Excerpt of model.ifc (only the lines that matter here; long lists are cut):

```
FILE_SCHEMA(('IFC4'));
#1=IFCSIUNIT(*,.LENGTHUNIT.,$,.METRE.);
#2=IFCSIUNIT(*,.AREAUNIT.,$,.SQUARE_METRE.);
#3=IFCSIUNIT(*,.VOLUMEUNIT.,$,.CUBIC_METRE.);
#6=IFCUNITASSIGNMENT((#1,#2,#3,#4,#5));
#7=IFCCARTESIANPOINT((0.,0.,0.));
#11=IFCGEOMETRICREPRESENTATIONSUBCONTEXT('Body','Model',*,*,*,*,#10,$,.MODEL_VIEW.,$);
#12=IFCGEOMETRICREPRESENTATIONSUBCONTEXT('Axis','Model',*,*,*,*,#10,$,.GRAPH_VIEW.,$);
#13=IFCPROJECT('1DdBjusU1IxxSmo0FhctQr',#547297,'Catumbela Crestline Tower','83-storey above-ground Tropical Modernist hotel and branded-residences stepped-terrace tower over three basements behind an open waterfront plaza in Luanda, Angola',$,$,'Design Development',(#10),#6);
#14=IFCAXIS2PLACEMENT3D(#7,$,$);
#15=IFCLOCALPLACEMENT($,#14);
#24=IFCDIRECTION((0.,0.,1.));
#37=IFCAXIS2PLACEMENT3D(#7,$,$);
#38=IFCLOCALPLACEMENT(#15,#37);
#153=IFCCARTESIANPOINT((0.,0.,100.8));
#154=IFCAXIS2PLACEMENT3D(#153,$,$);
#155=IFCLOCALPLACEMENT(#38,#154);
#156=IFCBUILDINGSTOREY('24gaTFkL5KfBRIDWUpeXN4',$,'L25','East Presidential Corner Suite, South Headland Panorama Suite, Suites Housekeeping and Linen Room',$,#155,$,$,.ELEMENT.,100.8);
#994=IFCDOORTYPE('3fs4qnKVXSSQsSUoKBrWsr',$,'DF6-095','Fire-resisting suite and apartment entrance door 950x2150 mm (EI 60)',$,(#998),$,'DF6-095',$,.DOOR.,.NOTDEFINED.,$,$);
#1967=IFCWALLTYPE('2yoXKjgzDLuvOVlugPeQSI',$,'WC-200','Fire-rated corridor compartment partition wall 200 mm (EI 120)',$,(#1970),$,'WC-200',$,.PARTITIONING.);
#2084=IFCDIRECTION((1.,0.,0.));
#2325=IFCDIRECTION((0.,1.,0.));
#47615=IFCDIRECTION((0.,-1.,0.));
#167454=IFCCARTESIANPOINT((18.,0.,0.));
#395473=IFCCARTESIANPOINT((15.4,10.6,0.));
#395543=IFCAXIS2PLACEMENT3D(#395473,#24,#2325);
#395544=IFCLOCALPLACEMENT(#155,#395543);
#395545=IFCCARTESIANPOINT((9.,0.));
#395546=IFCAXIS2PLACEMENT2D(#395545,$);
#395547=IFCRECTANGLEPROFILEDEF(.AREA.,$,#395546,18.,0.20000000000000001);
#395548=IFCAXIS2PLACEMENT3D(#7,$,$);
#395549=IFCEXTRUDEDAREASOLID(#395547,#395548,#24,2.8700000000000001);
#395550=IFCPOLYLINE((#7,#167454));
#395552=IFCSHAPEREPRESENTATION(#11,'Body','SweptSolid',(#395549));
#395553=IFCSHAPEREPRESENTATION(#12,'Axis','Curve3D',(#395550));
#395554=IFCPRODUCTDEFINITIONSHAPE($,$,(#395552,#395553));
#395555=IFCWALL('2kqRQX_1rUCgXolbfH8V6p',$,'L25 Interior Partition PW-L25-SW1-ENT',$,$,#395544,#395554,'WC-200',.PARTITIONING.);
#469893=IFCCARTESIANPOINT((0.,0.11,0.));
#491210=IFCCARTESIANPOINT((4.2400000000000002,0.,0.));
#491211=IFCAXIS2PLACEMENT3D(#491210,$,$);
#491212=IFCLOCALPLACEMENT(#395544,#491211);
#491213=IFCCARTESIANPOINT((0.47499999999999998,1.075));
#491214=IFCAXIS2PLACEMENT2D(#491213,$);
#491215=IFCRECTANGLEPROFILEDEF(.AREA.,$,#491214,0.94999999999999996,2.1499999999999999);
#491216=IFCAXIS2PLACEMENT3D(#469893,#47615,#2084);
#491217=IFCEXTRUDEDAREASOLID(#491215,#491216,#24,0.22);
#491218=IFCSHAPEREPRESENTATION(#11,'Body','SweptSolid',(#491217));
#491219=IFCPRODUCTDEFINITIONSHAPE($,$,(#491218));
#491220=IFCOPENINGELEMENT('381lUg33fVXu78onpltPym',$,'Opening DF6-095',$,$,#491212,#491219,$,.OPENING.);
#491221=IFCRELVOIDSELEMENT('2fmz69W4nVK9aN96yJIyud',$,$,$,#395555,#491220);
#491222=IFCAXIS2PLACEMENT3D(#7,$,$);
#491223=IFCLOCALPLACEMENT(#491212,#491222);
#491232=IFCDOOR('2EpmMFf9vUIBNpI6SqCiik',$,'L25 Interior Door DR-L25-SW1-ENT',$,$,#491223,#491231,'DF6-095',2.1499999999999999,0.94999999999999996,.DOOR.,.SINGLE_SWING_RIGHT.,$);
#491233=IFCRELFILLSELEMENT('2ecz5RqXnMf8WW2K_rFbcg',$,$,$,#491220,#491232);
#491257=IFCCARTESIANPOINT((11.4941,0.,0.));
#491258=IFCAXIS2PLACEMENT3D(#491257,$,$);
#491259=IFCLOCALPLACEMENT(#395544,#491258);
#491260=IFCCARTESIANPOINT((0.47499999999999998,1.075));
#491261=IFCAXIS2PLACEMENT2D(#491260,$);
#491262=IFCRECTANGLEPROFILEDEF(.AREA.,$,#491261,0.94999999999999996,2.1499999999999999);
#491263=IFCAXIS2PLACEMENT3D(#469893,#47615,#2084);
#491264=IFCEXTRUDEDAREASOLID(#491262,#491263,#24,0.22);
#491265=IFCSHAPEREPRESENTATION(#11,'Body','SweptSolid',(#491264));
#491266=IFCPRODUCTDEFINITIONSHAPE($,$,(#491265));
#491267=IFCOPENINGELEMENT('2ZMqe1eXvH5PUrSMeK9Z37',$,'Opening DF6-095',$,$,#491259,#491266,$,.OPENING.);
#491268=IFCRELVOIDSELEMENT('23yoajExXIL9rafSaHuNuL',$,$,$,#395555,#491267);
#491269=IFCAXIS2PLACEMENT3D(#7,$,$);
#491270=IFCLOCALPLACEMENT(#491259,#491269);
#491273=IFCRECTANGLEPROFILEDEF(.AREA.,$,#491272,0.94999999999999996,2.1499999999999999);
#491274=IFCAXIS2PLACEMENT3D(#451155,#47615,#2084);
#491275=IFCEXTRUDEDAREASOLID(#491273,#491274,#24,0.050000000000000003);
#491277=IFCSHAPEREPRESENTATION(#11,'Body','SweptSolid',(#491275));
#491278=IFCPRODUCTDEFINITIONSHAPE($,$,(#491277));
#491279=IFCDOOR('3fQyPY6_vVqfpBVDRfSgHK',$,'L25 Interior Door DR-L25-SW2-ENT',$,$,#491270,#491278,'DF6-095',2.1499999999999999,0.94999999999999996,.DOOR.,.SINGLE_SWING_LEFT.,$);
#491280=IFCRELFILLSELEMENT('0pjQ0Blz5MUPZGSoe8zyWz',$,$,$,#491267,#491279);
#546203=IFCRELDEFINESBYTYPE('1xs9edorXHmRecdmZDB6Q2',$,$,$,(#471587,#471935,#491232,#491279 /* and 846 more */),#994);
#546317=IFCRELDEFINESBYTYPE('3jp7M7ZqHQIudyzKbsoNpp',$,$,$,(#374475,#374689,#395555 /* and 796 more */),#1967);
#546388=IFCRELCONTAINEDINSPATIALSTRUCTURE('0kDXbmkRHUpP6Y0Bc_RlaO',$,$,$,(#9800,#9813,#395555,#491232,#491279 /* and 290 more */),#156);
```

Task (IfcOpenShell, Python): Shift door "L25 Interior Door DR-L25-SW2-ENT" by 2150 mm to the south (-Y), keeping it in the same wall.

```python
import ifcopenshell
import ifcopenshell.api.geometry
import ifcopenshell.util.placement

model = ifcopenshell.open("model.ifc")

door = model.by_guid("3fQyPY6_vVqfpBVDRfSgHK")
opening = door.FillsVoids[0].RelatingOpeningElement
wall = opening.VoidsElements[0].RelatingBuildingElement

wall_matrix = ifcopenshell.util.placement.get_local_placement(wall.ObjectPlacement)
shift = wall_matrix[:3, 0] * -2.15
before = ifcopenshell.util.placement.get_local_placement(door.ObjectPlacement)[:3, 3].copy()

# The door is placed relative to its opening, so it follows when the opening moves.
matrix = ifcopenshell.util.placement.get_local_placement(opening.ObjectPlacement)
matrix[:3, 3] += shift
ifcopenshell.api.geometry.edit_object_placement(
    model, product=opening, matrix=matrix, is_si=False, should_transform_children=True
)

after = ifcopenshell.util.placement.get_local_placement(door.ObjectPlacement)[:3, 3]
print("door moved by", (after - before).round(3) + 0.0)

model.write("model_edited.ifc")
```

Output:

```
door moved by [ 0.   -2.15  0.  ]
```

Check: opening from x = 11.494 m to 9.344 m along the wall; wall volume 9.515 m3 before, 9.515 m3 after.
